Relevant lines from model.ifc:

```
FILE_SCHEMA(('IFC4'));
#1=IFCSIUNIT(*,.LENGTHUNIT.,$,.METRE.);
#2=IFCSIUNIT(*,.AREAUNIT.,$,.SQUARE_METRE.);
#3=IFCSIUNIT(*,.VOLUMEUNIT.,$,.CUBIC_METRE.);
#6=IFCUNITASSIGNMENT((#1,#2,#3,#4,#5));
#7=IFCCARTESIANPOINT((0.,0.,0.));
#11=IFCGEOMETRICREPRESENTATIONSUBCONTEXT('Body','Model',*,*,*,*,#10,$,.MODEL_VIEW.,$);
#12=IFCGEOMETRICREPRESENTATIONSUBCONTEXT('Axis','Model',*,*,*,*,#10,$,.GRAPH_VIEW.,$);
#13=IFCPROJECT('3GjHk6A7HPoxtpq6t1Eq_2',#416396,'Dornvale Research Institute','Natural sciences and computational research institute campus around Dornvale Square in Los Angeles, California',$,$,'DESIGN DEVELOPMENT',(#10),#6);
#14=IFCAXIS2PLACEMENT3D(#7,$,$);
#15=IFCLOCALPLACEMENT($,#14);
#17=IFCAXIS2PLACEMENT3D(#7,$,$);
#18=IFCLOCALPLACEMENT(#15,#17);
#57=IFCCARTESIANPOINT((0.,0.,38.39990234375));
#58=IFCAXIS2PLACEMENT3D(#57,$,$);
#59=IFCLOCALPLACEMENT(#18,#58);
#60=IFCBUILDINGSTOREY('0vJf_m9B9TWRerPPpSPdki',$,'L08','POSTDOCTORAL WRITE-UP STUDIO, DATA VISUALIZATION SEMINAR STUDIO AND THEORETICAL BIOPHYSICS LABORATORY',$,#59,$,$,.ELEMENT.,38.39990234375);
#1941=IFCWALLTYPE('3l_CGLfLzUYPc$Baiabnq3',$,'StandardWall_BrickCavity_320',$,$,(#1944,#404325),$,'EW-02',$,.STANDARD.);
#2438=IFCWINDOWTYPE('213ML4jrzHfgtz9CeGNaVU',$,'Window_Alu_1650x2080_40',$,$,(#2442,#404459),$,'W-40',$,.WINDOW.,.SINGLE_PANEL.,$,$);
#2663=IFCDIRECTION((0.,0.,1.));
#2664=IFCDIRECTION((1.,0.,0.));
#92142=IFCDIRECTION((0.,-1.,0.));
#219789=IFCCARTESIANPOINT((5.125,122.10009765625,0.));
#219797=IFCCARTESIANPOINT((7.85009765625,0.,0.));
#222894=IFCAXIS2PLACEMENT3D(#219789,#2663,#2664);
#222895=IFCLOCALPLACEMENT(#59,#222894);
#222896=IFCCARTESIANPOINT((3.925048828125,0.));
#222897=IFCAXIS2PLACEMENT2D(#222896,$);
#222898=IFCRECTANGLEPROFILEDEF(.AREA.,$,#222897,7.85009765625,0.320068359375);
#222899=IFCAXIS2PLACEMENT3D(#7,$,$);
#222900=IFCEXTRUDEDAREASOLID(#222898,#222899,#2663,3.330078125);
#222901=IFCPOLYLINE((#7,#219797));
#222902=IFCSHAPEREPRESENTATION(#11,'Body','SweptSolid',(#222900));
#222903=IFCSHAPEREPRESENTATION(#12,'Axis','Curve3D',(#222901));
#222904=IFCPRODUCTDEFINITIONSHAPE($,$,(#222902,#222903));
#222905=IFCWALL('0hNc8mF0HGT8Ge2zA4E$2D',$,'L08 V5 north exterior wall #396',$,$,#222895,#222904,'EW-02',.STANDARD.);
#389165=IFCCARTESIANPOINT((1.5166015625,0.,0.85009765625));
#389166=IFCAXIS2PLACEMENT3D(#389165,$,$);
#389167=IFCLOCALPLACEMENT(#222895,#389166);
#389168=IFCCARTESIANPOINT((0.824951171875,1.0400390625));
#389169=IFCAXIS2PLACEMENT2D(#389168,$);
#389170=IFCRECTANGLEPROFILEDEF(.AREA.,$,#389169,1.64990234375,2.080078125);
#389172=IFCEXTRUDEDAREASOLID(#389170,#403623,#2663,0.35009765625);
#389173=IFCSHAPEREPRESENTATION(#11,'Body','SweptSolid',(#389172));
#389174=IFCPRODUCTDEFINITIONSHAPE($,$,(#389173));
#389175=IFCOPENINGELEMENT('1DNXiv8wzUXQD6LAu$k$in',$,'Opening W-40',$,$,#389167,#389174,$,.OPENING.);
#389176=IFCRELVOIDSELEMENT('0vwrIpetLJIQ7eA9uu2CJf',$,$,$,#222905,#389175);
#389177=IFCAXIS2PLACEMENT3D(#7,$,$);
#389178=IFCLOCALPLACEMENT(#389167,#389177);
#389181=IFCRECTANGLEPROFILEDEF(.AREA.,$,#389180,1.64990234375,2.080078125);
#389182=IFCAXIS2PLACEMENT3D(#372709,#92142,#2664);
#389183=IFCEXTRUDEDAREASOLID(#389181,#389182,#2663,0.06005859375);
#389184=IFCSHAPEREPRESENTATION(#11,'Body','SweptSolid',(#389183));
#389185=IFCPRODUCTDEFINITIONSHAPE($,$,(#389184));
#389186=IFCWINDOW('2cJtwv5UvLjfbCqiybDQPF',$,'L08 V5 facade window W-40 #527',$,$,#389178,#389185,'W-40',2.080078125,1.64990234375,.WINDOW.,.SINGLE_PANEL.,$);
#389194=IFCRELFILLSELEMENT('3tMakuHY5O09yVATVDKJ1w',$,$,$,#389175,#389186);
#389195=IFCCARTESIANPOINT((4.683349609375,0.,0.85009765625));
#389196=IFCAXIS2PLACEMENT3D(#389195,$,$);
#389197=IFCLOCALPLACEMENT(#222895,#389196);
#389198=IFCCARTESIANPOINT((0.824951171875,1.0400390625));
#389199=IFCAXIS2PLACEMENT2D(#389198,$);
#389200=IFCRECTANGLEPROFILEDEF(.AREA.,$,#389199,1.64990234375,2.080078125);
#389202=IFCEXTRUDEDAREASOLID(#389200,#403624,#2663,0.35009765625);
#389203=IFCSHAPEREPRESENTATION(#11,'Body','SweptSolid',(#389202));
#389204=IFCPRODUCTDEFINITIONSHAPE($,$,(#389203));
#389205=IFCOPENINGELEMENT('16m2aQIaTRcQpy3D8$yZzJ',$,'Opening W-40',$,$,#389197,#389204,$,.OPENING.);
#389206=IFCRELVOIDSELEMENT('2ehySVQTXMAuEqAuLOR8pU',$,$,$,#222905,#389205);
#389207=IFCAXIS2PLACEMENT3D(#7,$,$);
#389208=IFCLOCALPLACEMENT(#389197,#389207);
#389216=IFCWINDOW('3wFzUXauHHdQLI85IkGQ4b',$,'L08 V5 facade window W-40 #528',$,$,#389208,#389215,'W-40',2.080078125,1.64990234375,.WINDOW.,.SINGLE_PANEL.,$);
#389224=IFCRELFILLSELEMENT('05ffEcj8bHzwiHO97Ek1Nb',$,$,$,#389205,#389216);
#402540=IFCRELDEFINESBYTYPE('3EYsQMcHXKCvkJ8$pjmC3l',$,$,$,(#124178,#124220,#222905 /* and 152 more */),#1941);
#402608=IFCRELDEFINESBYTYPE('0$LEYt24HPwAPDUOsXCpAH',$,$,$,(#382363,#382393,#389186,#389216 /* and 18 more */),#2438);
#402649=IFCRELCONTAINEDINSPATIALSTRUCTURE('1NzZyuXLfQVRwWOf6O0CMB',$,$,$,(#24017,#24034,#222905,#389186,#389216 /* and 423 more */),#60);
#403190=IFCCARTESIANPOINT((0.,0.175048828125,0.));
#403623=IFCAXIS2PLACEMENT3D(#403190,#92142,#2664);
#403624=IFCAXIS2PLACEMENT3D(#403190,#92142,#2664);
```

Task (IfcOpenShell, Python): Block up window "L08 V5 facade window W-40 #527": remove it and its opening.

```python
import ifcopenshell
import ifcopenshell.api.feature
import ifcopenshell.api.root
import ifcopenshell.geom
import ifcopenshell.util.shape

model = ifcopenshell.open("model.ifc")
settings = ifcopenshell.geom.settings()


def volume(element):
    """Net volume in cubic metres, openings subtracted."""
    shape = ifcopenshell.geom.create_shape(settings, element)
    return ifcopenshell.util.shape.get_volume(shape.geometry)


window = model.by_guid("2cJtwv5UvLjfbCqiybDQPF")
opening = window.FillsVoids[0].RelatingOpeningElement
wall = opening.VoidsElements[0].RelatingBuildingElement
before = volume(wall)

ifcopenshell.api.root.remove_product(model, product=window)
ifcopenshell.api.feature.remove_feature(model, feature=opening)

after = volume(wall)

print(f"wall volume {before:.3f} -> {after:.3f} m3")

model.write("model_edited.ifc")
```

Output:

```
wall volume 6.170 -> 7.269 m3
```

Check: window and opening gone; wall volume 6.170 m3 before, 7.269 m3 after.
